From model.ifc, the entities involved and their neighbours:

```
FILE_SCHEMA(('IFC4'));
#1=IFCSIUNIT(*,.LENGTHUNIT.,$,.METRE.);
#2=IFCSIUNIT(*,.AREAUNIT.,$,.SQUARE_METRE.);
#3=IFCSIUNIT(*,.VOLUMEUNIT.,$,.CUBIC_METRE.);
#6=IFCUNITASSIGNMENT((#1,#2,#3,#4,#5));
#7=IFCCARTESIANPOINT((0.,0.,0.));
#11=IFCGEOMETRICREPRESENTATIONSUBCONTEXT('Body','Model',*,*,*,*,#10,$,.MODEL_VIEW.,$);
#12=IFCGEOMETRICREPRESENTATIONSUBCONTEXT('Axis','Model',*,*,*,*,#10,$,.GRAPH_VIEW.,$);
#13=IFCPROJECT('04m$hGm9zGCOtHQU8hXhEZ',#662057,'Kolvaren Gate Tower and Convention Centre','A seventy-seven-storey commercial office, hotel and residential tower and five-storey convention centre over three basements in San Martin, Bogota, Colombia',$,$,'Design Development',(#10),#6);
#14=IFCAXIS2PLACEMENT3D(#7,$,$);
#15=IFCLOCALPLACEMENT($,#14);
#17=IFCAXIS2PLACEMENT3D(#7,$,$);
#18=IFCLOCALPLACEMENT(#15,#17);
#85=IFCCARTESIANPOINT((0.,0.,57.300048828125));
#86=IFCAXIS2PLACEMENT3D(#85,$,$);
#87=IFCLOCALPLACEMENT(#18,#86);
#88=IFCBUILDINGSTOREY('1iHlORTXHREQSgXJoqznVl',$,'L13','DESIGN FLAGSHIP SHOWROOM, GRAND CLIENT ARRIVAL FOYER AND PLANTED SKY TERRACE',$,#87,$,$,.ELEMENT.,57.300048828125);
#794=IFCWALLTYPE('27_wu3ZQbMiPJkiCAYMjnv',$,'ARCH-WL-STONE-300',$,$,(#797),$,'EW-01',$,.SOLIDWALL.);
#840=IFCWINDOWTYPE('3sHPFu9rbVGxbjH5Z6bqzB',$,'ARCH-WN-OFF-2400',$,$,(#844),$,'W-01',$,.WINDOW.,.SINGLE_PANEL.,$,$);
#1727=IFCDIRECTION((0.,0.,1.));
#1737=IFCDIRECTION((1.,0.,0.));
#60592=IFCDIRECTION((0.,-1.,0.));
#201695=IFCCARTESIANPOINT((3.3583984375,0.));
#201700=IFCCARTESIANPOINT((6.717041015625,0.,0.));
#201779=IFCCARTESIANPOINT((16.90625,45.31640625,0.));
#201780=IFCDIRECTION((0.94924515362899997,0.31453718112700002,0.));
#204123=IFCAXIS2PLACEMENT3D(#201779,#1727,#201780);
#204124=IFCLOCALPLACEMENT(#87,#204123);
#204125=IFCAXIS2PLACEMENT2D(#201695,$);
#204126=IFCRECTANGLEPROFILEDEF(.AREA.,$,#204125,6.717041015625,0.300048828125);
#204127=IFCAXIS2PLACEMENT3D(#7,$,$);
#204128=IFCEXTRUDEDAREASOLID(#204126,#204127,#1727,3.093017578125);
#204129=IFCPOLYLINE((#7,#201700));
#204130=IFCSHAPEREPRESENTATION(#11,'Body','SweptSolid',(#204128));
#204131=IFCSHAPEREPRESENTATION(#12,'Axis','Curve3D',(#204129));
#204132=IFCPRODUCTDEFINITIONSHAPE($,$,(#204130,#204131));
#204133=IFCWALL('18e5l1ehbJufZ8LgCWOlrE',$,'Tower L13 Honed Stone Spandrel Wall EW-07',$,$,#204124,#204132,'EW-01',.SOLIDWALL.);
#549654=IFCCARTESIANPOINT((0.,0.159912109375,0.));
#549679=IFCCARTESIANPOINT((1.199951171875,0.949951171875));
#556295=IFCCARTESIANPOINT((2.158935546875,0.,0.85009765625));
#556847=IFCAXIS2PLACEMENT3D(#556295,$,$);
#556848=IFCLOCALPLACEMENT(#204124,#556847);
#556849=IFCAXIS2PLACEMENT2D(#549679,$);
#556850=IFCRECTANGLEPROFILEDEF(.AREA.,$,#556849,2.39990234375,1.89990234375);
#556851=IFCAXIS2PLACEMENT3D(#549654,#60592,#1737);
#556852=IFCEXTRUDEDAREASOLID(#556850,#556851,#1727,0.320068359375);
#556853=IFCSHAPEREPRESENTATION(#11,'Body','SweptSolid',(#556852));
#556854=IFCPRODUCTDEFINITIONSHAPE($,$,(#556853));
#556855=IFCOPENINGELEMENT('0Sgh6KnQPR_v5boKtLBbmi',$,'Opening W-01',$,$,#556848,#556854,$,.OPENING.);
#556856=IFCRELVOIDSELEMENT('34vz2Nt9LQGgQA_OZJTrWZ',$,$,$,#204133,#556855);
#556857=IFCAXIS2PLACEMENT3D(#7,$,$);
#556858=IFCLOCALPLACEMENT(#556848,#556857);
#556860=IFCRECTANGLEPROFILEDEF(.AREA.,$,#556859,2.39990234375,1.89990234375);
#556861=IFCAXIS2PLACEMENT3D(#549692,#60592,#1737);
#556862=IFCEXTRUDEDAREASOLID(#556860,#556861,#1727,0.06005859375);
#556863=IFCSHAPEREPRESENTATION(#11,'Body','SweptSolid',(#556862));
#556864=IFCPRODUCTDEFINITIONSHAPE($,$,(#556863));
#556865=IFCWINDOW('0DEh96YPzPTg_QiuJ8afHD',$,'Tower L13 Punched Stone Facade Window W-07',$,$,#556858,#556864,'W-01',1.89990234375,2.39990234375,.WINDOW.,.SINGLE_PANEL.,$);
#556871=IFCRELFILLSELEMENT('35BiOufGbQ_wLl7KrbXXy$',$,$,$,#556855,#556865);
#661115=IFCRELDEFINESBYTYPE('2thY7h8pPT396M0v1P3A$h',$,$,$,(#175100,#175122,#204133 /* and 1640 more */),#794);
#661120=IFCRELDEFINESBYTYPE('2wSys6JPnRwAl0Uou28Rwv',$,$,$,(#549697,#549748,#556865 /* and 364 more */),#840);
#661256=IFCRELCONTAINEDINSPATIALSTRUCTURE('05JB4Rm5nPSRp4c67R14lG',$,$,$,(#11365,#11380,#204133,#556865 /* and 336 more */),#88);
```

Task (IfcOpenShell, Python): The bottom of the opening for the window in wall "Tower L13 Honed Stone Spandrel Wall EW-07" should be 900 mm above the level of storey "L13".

```python
import numpy as np
import ifcopenshell
import ifcopenshell.api.geometry
import ifcopenshell.geom
import ifcopenshell.util.element
import ifcopenshell.util.placement
import ifcopenshell.util.shape
import ifcopenshell.util.unit

model = ifcopenshell.open("model.ifc")
unit_scale = ifcopenshell.util.unit.calculate_unit_scale(model)

window = model.by_id(556865)
opening = window.FillsVoids[0].RelatingOpeningElement
storey = ifcopenshell.util.element.get_container(window, ifc_class="IfcBuildingStorey")
level = ifcopenshell.util.placement.get_local_placement(storey.ObjectPlacement)[2, 3]

# The opening's origin need not be at the sill, so measure its lowest point.
shape = ifcopenshell.geom.create_shape(ifcopenshell.geom.settings(), opening)
bottom = ifcopenshell.util.shape.get_shape_bottom_elevation(shape, shape.geometry) / unit_scale
dz = level + 0.9 / unit_scale - bottom

shift = np.array([0.0, 0.0, dz])
# The window is placed relative to its opening, so it follows when the opening moves.
matrix = ifcopenshell.util.placement.get_local_placement(opening.ObjectPlacement)
matrix[:3, 3] += shift
ifcopenshell.api.geometry.edit_object_placement(
    model, product=opening, matrix=matrix, is_si=False, should_transform_children=True
)

print(f"moved by {dz * unit_scale:+.3f} m")

model.write("model_edited.ifc")
```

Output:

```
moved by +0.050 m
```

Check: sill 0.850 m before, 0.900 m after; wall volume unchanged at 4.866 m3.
